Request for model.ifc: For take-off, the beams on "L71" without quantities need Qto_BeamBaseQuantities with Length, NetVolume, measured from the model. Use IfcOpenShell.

First a look at what the model holds.

```python
import ifcopenshell
import ifcopenshell.util.element
import ifcopenshell.util.unit

model = ifcopenshell.open("model.ifc")
print(model.schema)
for unit_type in ("LENGTHUNIT", "AREAUNIT", "VOLUMEUNIT"):
    print(unit_type, ifcopenshell.util.unit.calculate_unit_scale(model, unit_type))
storey = next(s for s in model.by_type("IfcBuildingStorey") if s.Name == "L71")
beams = [e for e in ifcopenshell.util.element.get_decomposition(storey) if e.is_a("IfcBeam")]
for e in sorted(beams, key=lambda e: e.id()):
    print(e.id(), e.is_a(), e.Name, list(ifcopenshell.util.element.get_psets(e, qtos_only=True)), sep=" | ")
```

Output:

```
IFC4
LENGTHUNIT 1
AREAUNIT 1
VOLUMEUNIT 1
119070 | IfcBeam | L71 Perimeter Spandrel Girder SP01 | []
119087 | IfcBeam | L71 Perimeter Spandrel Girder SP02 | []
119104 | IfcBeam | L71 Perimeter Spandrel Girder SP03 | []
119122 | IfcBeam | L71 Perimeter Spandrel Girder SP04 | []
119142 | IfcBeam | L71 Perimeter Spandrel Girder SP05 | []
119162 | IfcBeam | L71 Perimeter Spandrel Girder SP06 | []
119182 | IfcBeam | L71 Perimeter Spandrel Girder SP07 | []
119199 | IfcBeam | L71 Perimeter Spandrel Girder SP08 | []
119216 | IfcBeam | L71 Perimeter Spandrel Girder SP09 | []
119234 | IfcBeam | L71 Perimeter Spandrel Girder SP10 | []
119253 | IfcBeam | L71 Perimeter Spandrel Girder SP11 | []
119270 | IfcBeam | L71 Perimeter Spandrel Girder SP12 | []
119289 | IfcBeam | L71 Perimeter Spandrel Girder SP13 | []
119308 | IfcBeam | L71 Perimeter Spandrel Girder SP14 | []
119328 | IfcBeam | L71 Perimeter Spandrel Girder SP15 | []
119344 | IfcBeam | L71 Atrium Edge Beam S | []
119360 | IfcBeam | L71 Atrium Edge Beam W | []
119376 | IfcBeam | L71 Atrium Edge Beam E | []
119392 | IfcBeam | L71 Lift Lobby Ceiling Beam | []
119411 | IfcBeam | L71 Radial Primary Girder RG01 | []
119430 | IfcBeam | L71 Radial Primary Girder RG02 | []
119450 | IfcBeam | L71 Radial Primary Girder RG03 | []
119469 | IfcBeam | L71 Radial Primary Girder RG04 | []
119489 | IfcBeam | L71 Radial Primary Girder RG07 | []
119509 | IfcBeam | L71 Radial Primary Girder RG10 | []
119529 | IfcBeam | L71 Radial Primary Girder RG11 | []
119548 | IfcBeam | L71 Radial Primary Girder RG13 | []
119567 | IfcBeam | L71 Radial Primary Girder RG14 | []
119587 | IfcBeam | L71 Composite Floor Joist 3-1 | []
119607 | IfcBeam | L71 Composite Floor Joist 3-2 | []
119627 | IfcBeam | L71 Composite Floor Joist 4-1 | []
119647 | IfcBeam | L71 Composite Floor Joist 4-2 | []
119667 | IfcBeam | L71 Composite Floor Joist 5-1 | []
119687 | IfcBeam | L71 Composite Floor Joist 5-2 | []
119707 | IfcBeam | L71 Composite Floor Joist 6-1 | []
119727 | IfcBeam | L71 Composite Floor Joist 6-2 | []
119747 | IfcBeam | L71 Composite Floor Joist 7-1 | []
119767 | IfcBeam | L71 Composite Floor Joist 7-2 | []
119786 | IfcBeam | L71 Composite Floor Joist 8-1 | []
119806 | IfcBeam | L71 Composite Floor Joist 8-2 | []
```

```python
import ifcopenshell
import ifcopenshell.api.pset
import ifcopenshell.geom
import ifcopenshell.util.element
import ifcopenshell.util.shape
import ifcopenshell.util.unit

model = ifcopenshell.open("model.ifc")
unit_scale = ifcopenshell.util.unit.calculate_unit_scale(model)
volume_scale = ifcopenshell.util.unit.calculate_unit_scale(model, "VOLUMEUNIT")
settings = ifcopenshell.geom.settings()

storey = next(s for s in model.by_type("IfcBuildingStorey") if s.Name == "L71")
beams = [e for e in ifcopenshell.util.element.get_decomposition(storey) if e.is_a("IfcBeam")]

for e in sorted(beams, key=lambda e: e.id()):
    if ifcopenshell.util.element.get_psets(e, qtos_only=True, should_inherit=False):
        continue
    # Geometry comes back in metres, in the element's own axes.
    shape = ifcopenshell.geom.create_shape(settings, e)
    values = {
        "Length": ifcopenshell.util.shape.get_max_xyz(shape.geometry) / unit_scale,
        "NetVolume": ifcopenshell.util.shape.get_volume(shape.geometry) / volume_scale,
    }
    qto = ifcopenshell.api.pset.add_qto(model, product=e, name="Qto_BeamBaseQuantities")
    ifcopenshell.api.pset.edit_qto(model, qto=qto, properties=values)
    print(e.id(), {k: round(v, 3) for k, v in values.items()})

model.write("model-out.ifc")
```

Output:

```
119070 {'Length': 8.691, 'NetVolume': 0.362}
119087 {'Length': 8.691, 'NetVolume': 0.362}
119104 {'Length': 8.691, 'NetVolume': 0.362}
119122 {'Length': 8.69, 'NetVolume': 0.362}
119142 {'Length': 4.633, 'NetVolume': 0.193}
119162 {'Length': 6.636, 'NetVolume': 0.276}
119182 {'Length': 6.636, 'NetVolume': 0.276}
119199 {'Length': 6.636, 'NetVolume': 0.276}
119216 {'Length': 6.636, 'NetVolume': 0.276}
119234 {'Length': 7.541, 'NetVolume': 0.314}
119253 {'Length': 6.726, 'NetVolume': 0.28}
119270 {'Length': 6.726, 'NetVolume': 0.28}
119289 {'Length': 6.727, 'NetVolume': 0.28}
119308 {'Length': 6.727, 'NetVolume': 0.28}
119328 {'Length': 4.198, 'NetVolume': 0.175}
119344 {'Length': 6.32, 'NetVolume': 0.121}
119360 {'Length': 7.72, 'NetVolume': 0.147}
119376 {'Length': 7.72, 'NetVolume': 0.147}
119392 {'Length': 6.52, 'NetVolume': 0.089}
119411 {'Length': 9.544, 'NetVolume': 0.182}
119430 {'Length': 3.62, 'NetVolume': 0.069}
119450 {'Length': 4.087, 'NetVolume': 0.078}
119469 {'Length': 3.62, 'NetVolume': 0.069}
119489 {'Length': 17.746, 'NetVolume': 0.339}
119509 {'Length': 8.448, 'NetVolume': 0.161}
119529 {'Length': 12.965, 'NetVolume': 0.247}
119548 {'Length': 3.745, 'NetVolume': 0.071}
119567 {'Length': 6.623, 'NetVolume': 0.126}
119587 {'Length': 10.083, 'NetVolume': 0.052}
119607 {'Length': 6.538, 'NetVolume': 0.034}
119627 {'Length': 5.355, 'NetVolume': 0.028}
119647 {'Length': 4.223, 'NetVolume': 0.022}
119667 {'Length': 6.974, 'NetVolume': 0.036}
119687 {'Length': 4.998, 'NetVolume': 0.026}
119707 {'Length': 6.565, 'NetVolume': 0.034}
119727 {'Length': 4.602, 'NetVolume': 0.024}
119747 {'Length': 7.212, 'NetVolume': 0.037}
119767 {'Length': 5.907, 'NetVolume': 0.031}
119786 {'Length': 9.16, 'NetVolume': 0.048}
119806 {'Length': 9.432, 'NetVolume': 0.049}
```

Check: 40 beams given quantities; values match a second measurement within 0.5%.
